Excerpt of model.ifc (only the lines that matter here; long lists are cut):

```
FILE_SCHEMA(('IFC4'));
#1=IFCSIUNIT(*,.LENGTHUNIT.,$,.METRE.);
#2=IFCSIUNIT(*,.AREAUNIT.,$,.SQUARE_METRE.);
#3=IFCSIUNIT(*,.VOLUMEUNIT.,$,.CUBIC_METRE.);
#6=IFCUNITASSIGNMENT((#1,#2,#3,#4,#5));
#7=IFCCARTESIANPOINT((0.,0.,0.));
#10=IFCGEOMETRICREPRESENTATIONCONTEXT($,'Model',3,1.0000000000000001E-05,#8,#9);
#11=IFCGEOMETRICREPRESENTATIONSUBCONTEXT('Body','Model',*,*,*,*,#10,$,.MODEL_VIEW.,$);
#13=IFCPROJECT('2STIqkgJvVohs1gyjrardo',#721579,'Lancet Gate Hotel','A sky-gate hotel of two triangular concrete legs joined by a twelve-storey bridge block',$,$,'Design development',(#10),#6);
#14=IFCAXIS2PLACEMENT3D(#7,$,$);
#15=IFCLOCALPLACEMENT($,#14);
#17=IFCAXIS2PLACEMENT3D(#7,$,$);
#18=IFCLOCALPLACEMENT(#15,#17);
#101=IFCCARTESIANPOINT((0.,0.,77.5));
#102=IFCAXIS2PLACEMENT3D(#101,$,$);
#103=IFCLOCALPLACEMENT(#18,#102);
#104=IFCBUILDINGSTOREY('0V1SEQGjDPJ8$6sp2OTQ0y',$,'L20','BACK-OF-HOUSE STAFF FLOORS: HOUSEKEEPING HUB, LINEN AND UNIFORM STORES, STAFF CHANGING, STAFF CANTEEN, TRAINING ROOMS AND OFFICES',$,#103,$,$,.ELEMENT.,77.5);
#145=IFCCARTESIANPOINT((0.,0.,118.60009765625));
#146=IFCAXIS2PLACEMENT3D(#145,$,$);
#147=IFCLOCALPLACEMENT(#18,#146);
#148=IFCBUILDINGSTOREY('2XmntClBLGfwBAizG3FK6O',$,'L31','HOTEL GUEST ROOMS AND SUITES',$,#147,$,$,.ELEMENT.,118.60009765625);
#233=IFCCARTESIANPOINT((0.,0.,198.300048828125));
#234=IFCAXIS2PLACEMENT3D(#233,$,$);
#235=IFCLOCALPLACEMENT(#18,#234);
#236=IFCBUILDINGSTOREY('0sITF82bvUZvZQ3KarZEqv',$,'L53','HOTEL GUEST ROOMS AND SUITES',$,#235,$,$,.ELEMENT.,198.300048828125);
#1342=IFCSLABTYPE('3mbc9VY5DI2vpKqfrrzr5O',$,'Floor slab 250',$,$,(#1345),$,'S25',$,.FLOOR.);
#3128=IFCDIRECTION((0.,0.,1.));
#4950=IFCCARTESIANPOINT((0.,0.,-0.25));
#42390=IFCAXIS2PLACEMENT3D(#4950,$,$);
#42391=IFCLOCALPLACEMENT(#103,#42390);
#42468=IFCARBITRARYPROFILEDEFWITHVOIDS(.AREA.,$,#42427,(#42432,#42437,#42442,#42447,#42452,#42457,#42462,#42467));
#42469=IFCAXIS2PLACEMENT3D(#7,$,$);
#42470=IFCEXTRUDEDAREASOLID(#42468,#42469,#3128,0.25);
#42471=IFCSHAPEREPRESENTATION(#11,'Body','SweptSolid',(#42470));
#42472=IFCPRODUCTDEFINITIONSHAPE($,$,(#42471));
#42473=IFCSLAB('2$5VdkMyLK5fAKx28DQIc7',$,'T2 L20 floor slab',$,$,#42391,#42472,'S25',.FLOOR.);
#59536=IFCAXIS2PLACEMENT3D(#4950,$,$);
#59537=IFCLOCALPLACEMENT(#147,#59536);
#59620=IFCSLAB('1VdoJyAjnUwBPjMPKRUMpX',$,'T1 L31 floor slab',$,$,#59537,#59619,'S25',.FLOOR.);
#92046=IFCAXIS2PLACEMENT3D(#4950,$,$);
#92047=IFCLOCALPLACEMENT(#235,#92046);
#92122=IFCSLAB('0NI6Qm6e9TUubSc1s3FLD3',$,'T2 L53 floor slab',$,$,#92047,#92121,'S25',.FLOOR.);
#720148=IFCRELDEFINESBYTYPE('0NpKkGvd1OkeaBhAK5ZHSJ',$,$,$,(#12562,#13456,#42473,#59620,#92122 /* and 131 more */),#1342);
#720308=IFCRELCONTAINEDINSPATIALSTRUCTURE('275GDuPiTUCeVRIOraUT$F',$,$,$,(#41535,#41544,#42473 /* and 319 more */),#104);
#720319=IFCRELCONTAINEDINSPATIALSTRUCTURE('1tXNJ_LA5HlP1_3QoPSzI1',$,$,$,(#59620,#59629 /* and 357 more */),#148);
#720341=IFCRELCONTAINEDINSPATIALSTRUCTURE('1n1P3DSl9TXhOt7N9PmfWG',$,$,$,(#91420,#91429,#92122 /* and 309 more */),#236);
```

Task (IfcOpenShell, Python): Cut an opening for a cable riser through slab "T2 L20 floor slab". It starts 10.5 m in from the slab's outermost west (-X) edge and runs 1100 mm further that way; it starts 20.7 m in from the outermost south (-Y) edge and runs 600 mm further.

```python
import numpy as np
import ifcopenshell
import ifcopenshell.api.feature
import ifcopenshell.api.geometry
import ifcopenshell.api.root
import ifcopenshell.geom
import ifcopenshell.util.placement
import ifcopenshell.util.representation
import ifcopenshell.util.shape
import ifcopenshell.util.unit

model = ifcopenshell.open("model.ifc")
unit_scale = ifcopenshell.util.unit.calculate_unit_scale(model)
settings = ifcopenshell.geom.settings()


def volume(element):
    """Net volume in cubic metres, openings subtracted."""
    shape = ifcopenshell.geom.create_shape(settings, element)
    return ifcopenshell.util.shape.get_volume(shape.geometry)


slab = model.by_guid("2$5VdkMyLK5fAKx28DQIc7")
before = volume(slab)

# Extent in the slab's own axes, in metres. The edges named are its -X and -Y sides.
slab_shape = ifcopenshell.geom.create_shape(settings, slab)
vertices = ifcopenshell.util.shape.get_vertices(slab_shape.geometry)
x_min, y_min, bottom = vertices.min(axis=0)
top = vertices[:, 2].max()

opening = ifcopenshell.api.root.create_entity(model, ifc_class="IfcOpeningElement", name="Cable riser opening", predefined_type="OPENING")
context = ifcopenshell.util.representation.get_context(model, "Model", "Body", "MODEL_VIEW")
width, depth = 1.1, 0.6
outline = [(0.0, 0.0), (width, 0.0), (width, depth), (0.0, depth), (0.0, 0.0)]
# Overshoot both faces by 50 mm so the cut is clean.
shape = ifcopenshell.api.geometry.add_slab_representation(
    model, context=context, depth=top - bottom + 0.1, polyline=outline
)
ifcopenshell.api.geometry.assign_representation(model, product=opening, representation=shape)

matrix = ifcopenshell.util.placement.get_local_placement(slab.ObjectPlacement)
matrix[:, 3] = matrix @ np.append(np.array([x_min + 10.5, y_min + 20.7, bottom - 0.05]) / unit_scale, 1.0)
ifcopenshell.api.geometry.edit_object_placement(model, product=opening, matrix=matrix, is_si=False)
ifcopenshell.api.feature.add_feature(model, feature=opening, element=slab)

after = volume(slab)

print(f"slab volume {before:.3f} -> {after:.3f} m3")

model.write("model_v2.ifc")
```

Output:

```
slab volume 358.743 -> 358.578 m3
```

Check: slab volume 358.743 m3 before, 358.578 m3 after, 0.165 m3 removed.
